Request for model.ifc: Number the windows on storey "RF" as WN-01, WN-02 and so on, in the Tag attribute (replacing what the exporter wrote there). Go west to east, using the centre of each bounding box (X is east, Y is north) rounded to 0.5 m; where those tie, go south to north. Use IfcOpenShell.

First a look at what the model holds.

```python
import ifcopenshell
import ifcopenshell.util.element
import ifcopenshell.util.placement

model = ifcopenshell.open("model.ifc")
print(model.schema)
storey = next(s for s in model.by_type("IfcBuildingStorey") if s.Name == "RF")
windows = [e for e in ifcopenshell.util.element.get_decomposition(storey) if e.is_a("IfcWindow")]
for e in sorted(windows, key=lambda e: e.id()):
    origin = ifcopenshell.util.placement.get_local_placement(e.ObjectPlacement)[:3, 3]
    print(e.id(), e.Tag, e.Name, origin.round(2) + 0.0, sep=" | ")
```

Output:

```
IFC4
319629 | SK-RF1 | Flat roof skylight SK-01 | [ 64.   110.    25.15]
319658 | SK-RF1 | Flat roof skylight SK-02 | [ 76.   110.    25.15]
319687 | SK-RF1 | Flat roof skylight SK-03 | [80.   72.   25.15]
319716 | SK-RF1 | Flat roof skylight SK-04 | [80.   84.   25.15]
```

```python
import ifcopenshell
import ifcopenshell.geom
import ifcopenshell.util.element
import ifcopenshell.util.shape

model = ifcopenshell.open("model.ifc")
settings = ifcopenshell.geom.settings()
settings.set("use-world-coords", True)


def centre(element):
    shape = ifcopenshell.geom.create_shape(settings, element)
    return ifcopenshell.util.shape.get_bbox_centroid(shape.geometry)


storey = next(s for s in model.by_type("IfcBuildingStorey") if s.Name == "RF")
windows = [e for e in ifcopenshell.util.element.get_decomposition(storey) if e.is_a("IfcWindow")]

# Insertion points can sit at a corner or the storey origin, so sort by the geometry (in metres).
centres = {e: centre(e) for e in windows}
windows.sort(key=lambda e: (round(centres[e][0] / 0.5), centres[e][1]))

for i, e in enumerate(windows, start=1):
    number = f"WN-{i:02d}"
    e.Tag = number
    print(e.id(), number)

model.write("model_updated.ifc")
```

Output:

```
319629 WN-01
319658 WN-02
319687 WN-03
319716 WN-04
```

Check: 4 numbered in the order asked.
